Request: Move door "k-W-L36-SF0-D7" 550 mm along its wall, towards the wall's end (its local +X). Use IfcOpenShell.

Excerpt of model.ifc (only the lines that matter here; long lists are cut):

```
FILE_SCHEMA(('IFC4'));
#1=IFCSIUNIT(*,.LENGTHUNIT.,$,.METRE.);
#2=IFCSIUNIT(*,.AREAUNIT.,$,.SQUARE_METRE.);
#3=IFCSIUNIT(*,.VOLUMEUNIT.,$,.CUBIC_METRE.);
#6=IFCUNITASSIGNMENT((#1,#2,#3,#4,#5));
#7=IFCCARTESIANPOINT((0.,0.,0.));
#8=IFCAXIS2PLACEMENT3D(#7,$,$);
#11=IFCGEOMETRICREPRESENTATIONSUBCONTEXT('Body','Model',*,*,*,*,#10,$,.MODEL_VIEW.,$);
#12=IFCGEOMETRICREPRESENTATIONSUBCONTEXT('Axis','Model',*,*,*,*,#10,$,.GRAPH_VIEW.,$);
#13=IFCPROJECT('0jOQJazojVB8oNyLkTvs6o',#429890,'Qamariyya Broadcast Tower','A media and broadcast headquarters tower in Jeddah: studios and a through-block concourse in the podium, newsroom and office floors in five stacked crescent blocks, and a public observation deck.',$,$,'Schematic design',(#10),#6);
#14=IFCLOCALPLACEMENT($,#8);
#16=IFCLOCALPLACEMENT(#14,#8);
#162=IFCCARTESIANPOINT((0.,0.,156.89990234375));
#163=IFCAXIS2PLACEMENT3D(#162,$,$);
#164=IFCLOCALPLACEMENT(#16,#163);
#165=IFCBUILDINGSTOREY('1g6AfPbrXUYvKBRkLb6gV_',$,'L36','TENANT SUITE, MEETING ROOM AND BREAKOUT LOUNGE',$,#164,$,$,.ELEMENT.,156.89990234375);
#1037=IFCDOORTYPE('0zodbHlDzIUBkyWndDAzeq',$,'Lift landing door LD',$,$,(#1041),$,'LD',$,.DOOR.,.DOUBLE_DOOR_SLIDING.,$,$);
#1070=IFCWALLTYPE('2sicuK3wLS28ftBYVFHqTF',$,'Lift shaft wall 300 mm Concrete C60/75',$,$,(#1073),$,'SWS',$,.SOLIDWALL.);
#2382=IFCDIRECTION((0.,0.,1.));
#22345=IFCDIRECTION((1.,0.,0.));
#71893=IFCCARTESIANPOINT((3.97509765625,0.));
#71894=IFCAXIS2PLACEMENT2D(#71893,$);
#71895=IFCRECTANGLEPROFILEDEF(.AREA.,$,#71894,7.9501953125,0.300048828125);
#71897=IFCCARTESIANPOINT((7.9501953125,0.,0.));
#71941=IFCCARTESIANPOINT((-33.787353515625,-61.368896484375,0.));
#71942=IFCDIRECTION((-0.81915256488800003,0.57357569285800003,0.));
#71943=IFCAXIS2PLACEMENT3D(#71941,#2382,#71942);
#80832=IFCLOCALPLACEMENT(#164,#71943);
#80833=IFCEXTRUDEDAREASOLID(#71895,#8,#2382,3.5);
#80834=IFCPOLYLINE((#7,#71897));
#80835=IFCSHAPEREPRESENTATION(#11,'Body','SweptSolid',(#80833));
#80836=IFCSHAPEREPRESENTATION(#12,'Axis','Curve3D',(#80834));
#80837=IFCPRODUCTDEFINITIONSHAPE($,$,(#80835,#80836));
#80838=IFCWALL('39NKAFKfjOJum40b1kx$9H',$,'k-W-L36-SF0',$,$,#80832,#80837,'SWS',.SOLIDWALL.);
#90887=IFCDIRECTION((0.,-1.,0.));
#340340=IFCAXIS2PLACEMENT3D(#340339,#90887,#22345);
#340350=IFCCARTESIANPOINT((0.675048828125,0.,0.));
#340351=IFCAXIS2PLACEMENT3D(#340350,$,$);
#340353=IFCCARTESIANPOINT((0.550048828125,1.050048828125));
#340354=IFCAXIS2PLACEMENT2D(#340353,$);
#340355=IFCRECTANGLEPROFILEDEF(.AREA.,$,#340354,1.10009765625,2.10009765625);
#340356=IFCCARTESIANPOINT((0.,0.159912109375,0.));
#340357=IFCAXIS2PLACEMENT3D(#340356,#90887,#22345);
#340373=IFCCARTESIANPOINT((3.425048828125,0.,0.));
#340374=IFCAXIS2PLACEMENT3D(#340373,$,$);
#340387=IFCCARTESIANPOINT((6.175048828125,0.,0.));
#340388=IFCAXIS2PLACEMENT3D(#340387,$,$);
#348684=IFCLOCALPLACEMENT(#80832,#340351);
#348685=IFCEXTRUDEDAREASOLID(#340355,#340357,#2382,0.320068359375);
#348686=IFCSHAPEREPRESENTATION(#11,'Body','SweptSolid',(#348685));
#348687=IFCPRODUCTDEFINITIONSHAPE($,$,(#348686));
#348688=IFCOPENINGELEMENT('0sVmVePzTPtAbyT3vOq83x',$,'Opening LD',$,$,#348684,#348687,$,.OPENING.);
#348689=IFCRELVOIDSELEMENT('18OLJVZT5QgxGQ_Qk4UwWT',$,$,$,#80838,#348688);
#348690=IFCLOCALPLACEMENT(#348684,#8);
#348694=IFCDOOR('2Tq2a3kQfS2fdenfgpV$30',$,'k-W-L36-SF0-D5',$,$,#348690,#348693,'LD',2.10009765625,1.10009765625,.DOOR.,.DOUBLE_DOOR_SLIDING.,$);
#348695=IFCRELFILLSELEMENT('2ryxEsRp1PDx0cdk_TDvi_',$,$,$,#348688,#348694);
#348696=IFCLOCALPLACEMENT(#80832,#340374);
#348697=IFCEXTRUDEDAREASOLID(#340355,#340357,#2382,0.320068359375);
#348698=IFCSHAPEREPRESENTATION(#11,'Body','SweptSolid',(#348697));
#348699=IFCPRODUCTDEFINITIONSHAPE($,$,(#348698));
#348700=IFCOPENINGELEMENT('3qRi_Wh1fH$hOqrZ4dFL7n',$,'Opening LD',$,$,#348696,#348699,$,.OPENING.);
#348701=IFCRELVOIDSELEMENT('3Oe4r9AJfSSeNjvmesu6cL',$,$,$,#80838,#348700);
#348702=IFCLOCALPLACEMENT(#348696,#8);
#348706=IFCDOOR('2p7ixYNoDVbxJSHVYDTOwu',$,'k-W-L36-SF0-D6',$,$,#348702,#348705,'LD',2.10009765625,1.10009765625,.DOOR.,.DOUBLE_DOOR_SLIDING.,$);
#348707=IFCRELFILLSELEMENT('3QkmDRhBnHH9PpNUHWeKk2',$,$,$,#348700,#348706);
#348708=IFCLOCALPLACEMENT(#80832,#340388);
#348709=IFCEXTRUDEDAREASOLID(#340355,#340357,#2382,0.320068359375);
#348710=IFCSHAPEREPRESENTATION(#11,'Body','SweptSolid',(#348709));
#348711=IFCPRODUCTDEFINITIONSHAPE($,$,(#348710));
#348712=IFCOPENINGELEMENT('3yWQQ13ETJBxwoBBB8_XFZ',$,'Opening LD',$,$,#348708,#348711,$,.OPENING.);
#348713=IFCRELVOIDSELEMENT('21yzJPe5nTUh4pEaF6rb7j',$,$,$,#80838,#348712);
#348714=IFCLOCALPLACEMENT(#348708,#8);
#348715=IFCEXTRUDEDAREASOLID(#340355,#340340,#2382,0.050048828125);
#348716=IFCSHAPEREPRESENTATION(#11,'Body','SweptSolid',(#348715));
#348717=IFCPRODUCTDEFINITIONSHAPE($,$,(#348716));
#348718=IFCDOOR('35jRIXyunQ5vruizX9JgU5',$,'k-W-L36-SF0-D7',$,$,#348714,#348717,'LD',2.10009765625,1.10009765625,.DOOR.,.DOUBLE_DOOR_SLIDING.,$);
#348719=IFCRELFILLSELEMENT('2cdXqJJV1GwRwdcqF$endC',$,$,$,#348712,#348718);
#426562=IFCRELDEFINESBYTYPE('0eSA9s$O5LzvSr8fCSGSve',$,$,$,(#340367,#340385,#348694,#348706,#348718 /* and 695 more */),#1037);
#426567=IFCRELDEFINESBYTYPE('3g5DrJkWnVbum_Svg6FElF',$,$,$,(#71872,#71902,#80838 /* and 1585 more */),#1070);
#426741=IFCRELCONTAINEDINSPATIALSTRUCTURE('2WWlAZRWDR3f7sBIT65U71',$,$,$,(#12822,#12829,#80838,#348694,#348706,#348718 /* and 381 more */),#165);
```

```python
import ifcopenshell
import ifcopenshell.api.geometry
import ifcopenshell.util.placement

model = ifcopenshell.open("model.ifc")

door = model.by_id(348718)
opening = door.FillsVoids[0].RelatingOpeningElement
wall = opening.VoidsElements[0].RelatingBuildingElement

wall_matrix = ifcopenshell.util.placement.get_local_placement(wall.ObjectPlacement)
shift = wall_matrix[:3, 0] * 0.55
before = ifcopenshell.util.placement.get_local_placement(door.ObjectPlacement)[:3, 3].copy()

# The door is placed relative to its opening, so it follows when the opening moves.
matrix = ifcopenshell.util.placement.get_local_placement(opening.ObjectPlacement)
matrix[:3, 3] += shift
ifcopenshell.api.geometry.edit_object_placement(
    model, product=opening, matrix=matrix, is_si=False, should_transform_children=True
)

after = ifcopenshell.util.placement.get_local_placement(door.ObjectPlacement)[:3, 3]
print("door moved by", (after - before).round(3) + 0.0)

model.write("model_rev.ifc")
```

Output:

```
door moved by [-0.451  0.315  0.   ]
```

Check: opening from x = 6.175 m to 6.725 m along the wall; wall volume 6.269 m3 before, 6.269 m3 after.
